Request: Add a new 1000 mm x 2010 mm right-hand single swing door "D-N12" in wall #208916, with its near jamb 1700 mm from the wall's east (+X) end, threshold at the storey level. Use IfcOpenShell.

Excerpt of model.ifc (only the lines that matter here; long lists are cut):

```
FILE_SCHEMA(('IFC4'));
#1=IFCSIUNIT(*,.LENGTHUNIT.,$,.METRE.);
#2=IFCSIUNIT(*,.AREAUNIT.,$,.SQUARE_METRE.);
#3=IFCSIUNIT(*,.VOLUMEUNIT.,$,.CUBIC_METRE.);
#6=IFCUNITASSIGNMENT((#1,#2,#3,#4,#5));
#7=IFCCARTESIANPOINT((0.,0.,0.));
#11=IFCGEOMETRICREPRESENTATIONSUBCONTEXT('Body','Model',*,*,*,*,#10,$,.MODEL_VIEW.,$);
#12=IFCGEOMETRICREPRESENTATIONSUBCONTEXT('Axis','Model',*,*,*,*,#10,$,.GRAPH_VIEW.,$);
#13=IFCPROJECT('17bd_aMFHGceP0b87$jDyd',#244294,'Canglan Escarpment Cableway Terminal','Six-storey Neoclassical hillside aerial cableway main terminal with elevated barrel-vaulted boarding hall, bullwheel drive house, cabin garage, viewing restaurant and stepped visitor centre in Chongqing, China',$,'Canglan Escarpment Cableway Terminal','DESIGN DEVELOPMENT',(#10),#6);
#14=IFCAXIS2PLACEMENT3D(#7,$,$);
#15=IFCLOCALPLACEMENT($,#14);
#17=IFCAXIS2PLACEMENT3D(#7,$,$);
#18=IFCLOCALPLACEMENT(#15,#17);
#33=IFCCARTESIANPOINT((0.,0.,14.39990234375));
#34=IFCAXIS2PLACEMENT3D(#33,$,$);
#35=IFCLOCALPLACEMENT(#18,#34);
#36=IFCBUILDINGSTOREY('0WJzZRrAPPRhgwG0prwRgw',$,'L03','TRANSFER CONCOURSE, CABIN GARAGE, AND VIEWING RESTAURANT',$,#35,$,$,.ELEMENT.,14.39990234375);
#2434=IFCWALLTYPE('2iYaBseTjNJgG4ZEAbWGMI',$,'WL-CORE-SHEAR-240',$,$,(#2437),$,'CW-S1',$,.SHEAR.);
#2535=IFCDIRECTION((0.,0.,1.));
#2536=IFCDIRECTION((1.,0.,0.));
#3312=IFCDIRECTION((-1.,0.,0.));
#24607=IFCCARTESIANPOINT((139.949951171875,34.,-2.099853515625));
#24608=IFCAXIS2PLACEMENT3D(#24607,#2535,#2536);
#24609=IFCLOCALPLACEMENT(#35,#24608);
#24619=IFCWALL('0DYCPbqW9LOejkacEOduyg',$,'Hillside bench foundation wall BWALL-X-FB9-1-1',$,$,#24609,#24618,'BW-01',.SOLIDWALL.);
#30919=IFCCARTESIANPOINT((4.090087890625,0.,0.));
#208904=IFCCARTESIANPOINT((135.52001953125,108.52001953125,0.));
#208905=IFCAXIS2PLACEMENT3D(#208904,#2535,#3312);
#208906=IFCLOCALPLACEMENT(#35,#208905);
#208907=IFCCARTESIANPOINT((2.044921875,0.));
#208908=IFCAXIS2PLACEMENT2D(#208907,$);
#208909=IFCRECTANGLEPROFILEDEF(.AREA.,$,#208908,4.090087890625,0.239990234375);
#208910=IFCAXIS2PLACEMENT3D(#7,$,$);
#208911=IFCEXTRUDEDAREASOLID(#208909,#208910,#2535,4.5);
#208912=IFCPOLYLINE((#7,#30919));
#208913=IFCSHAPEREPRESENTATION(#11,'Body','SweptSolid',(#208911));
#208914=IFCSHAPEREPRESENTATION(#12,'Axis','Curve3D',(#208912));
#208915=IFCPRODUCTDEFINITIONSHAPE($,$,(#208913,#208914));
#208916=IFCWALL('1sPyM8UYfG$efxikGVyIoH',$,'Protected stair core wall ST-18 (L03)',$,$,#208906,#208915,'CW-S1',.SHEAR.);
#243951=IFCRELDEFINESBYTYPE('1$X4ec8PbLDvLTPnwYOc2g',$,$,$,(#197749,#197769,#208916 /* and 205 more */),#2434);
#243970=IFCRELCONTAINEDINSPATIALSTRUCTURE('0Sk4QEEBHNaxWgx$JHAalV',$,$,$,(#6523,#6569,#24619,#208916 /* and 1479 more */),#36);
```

```python
import numpy as np
import ifcopenshell
import ifcopenshell.api.feature
import ifcopenshell.api.geometry
import ifcopenshell.api.root
import ifcopenshell.api.spatial
import ifcopenshell.geom
import ifcopenshell.util.element
import ifcopenshell.util.placement
import ifcopenshell.util.representation
import ifcopenshell.util.shape
import ifcopenshell.util.unit

model = ifcopenshell.open("model.ifc")
unit_scale = ifcopenshell.util.unit.calculate_unit_scale(model)
settings = ifcopenshell.geom.settings()


def volume(element):
    """Net volume in cubic metres, openings subtracted."""
    shape = ifcopenshell.geom.create_shape(settings, element)
    return ifcopenshell.util.shape.get_volume(shape.geometry)


wall = model.by_id(208916)
storey = ifcopenshell.util.element.get_container(wall, ifc_class="IfcBuildingStorey")
context = ifcopenshell.util.representation.get_context(model, "Model", "Body", "MODEL_VIEW")
before = volume(wall)

width, height, from_end, sill = 1, 2.01, 1.7, 0.0  # metres

# The wall runs along its own X axis, and the end named is its -X end.
wall_shape = ifcopenshell.geom.create_shape(settings, wall)
x, y, z = ifcopenshell.util.shape.get_vertices(wall_shape.geometry).T
start = x.min() + from_end
face, thickness = float(y.min()), float(y.max() - y.min())
wall_matrix = ifcopenshell.util.placement.get_local_placement(wall.ObjectPlacement)
level = ifcopenshell.util.placement.get_local_placement(storey.ObjectPlacement)[2, 3]


def in_wall(x, y):
    """Placement at x, y metres in the wall's axes, at sill height."""
    matrix = wall_matrix.copy()
    matrix[:, 3] = wall_matrix @ np.array([x / unit_scale, y / unit_scale, 0.0, 1.0])
    matrix[2, 3] = level + sill / unit_scale
    return matrix


# Opening: a box that overshoots both wall faces by 50 mm.
opening = ifcopenshell.api.root.create_entity(model, ifc_class="IfcOpeningElement", predefined_type="OPENING")
box = ifcopenshell.api.geometry.add_wall_representation(
    model, context=context, length=width, height=height, thickness=thickness + 0.1
)
ifcopenshell.api.geometry.assign_representation(model, product=opening, representation=box)
ifcopenshell.api.geometry.edit_object_placement(model, product=opening, matrix=in_wall(start, face - 0.05), is_si=False)
ifcopenshell.api.feature.add_feature(model, feature=opening, element=wall)

door = ifcopenshell.api.root.create_entity(model, ifc_class="IfcDoor", name="D-N12", predefined_type="DOOR")
door.OverallWidth, door.OverallHeight = width / unit_scale, height / unit_scale
door.OperationType = "SINGLE_SWING_RIGHT"
body = ifcopenshell.api.geometry.add_door_representation(
    model,
    context=context,
    overall_width=door.OverallWidth,
    overall_height=door.OverallHeight,
    operation_type="SINGLE_SWING_RIGHT",
    lining_properties={"LiningDepth": thickness / unit_scale, "ThresholdDepth": thickness / unit_scale},
)
ifcopenshell.api.geometry.assign_representation(model, product=door, representation=body)
ifcopenshell.api.spatial.assign_container(model, products=[door], relating_structure=storey)
ifcopenshell.api.feature.add_filling(model, opening=opening, element=door)

# The lining spans the wall, so the door starts at the wall face.
ifcopenshell.api.geometry.edit_object_placement(model, product=door, matrix=in_wall(start, face), is_si=False)

after = volume(wall)

print(f"wall volume {before:.3f} -> {after:.3f} m3")

model.write("model-out.ifc")
```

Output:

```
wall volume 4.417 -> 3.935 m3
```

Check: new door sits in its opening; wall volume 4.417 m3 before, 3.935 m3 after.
